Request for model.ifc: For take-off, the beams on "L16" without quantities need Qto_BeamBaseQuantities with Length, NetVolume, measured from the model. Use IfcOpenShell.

First a look at what the model holds.

```python
import ifcopenshell
import ifcopenshell.util.element
import ifcopenshell.util.unit

model = ifcopenshell.open("model.ifc")
print(model.schema)
for unit_type in ("LENGTHUNIT", "AREAUNIT", "VOLUMEUNIT"):
    print(unit_type, ifcopenshell.util.unit.calculate_unit_scale(model, unit_type))
storey = next(s for s in model.by_type("IfcBuildingStorey") if s.Name == "L16")
beams = [e for e in ifcopenshell.util.element.get_decomposition(storey) if e.is_a("IfcBeam")]
for e in sorted(beams, key=lambda e: e.id()):
    print(e.id(), e.is_a(), e.Name, list(ifcopenshell.util.element.get_psets(e, qtos_only=True)), sep=" | ")
```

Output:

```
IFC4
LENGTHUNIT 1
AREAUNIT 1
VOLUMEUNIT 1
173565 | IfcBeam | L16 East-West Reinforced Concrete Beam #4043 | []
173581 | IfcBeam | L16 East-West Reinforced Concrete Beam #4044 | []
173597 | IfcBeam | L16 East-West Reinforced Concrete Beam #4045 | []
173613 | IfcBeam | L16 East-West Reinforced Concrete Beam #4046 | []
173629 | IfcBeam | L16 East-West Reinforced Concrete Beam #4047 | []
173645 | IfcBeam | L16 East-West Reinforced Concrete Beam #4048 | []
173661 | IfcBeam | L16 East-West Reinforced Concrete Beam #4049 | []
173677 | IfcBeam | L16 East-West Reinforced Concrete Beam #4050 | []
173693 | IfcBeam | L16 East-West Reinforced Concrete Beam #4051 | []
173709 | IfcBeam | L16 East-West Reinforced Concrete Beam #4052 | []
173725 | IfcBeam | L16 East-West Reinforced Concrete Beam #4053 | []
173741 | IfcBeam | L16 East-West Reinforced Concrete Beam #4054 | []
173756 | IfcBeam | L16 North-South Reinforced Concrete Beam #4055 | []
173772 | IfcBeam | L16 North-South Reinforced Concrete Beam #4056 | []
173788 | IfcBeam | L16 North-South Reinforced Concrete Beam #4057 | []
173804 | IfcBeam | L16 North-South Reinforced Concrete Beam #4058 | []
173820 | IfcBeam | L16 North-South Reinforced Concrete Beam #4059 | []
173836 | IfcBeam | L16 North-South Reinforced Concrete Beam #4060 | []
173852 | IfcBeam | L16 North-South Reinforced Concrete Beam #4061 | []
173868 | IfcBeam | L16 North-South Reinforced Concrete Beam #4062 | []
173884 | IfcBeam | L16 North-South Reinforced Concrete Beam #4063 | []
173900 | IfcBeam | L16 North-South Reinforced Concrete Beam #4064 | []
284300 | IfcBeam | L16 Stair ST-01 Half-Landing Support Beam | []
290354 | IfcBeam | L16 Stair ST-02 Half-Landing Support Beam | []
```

```python
import ifcopenshell
import ifcopenshell.api.pset
import ifcopenshell.geom
import ifcopenshell.util.element
import ifcopenshell.util.shape
import ifcopenshell.util.unit

model = ifcopenshell.open("model.ifc")
unit_scale = ifcopenshell.util.unit.calculate_unit_scale(model)
volume_scale = ifcopenshell.util.unit.calculate_unit_scale(model, "VOLUMEUNIT")
settings = ifcopenshell.geom.settings()

storey = next(s for s in model.by_type("IfcBuildingStorey") if s.Name == "L16")
beams = [e for e in ifcopenshell.util.element.get_decomposition(storey) if e.is_a("IfcBeam")]

for e in sorted(beams, key=lambda e: e.id()):
    if ifcopenshell.util.element.get_psets(e, qtos_only=True, should_inherit=False):
        continue
    # Geometry comes back in metres, in the element's own axes.
    shape = ifcopenshell.geom.create_shape(settings, e)
    values = {
        "Length": ifcopenshell.util.shape.get_max_xyz(shape.geometry) / unit_scale,
        "NetVolume": ifcopenshell.util.shape.get_volume(shape.geometry) / volume_scale,
    }
    qto = ifcopenshell.api.pset.add_qto(model, product=e, name="Qto_BeamBaseQuantities")
    ifcopenshell.api.pset.edit_qto(model, qto=qto, properties=values)
    print(e.id(), {k: round(v, 3) for k, v in values.items()})

model.write("model_updated.ifc")
```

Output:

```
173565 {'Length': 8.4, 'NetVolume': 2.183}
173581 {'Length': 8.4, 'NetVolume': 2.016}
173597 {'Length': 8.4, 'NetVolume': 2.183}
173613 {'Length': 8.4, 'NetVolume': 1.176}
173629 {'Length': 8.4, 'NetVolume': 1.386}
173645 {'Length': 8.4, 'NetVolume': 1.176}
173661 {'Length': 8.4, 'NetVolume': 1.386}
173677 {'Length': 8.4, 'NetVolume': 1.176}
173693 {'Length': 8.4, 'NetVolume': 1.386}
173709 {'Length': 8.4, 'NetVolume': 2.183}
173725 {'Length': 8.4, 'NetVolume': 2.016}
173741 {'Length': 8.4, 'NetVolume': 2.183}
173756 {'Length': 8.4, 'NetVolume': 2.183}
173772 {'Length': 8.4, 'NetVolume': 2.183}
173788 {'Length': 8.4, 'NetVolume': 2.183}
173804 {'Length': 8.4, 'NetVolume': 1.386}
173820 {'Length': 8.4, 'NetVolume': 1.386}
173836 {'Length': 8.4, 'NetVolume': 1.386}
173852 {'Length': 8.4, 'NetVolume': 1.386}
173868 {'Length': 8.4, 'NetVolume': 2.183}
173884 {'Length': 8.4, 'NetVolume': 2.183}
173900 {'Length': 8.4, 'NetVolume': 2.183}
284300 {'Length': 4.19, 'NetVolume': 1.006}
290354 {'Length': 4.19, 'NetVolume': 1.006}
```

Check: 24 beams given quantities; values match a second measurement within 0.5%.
